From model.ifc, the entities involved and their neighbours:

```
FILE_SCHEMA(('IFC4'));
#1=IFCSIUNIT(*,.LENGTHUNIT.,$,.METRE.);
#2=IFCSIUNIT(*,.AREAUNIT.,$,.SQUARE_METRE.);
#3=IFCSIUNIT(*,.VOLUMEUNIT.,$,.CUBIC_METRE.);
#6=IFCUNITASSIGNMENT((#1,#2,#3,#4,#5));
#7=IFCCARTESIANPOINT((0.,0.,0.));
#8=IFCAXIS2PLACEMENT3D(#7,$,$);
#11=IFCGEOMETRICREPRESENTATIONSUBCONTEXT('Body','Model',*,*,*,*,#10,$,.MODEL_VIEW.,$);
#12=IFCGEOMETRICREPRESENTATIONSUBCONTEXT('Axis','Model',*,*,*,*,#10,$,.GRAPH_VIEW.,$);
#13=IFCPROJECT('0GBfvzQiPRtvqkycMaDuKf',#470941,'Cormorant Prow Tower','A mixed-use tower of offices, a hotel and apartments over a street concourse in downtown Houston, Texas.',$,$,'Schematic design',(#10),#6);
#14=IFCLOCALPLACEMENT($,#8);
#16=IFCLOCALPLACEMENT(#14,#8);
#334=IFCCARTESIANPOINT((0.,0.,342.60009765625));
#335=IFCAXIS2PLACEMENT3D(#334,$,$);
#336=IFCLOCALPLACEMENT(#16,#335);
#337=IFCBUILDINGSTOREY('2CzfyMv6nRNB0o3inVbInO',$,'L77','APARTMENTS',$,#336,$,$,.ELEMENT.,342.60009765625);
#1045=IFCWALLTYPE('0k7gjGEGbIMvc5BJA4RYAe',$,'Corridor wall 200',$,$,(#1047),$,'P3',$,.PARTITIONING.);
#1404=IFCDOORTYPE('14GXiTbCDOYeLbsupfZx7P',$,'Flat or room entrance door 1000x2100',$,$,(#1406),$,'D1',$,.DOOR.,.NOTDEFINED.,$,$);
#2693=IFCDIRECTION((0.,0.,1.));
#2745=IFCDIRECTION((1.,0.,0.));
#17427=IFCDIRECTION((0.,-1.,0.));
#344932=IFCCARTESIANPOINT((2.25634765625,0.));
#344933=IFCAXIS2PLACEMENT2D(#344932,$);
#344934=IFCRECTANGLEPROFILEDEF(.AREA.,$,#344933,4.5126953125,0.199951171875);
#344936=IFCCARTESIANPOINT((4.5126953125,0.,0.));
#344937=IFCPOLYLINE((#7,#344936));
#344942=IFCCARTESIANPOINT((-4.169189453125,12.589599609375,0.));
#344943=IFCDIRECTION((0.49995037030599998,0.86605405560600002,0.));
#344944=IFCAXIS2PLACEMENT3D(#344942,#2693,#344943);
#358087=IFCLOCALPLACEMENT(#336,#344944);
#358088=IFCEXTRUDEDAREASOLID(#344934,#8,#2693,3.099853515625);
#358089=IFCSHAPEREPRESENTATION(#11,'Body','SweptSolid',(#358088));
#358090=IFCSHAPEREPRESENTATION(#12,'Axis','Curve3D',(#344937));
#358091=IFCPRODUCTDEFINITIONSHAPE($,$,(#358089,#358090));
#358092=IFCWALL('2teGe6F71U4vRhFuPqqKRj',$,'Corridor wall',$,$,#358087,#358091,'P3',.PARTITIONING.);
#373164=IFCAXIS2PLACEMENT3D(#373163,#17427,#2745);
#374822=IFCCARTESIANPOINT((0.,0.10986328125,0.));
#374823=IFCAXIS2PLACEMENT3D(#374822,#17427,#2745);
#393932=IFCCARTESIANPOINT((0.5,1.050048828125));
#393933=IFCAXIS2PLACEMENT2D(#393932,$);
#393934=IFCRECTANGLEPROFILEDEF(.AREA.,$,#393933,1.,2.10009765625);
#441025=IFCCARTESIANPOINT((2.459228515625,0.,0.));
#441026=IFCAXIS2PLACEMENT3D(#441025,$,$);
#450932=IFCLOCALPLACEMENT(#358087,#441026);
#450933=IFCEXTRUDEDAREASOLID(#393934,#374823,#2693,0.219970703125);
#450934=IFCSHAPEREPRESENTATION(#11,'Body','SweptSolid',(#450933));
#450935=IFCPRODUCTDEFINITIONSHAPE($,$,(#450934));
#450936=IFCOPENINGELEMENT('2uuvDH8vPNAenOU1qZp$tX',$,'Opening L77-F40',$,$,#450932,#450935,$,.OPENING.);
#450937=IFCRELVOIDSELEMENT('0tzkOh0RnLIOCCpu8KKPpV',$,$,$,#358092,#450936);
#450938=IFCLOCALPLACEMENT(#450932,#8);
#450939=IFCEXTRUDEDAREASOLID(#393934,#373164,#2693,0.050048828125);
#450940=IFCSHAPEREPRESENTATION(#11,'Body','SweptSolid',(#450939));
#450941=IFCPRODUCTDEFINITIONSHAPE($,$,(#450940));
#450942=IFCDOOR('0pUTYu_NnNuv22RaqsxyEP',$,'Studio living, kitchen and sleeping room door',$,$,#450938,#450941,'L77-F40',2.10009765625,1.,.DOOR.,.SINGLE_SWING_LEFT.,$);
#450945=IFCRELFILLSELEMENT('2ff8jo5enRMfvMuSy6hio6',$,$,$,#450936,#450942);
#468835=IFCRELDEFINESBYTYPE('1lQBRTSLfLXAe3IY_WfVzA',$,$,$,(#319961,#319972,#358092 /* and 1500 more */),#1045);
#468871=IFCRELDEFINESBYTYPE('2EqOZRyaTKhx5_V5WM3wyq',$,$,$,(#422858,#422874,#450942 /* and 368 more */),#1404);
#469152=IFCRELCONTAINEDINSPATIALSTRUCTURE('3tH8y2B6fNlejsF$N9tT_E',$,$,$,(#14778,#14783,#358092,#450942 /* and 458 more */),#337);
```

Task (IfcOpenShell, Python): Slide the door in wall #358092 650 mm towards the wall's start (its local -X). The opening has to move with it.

```python
import ifcopenshell
import ifcopenshell.api.geometry
import ifcopenshell.util.placement

model = ifcopenshell.open("model.ifc")

door = model.by_id(450942)
opening = door.FillsVoids[0].RelatingOpeningElement
wall = opening.VoidsElements[0].RelatingBuildingElement

wall_matrix = ifcopenshell.util.placement.get_local_placement(wall.ObjectPlacement)
shift = wall_matrix[:3, 0] * -0.65
before = ifcopenshell.util.placement.get_local_placement(door.ObjectPlacement)[:3, 3].copy()

# The door is placed relative to its opening, so it follows when the opening moves.
matrix = ifcopenshell.util.placement.get_local_placement(opening.ObjectPlacement)
matrix[:3, 3] += shift
ifcopenshell.api.geometry.edit_object_placement(
    model, product=opening, matrix=matrix, is_si=False, should_transform_children=True
)

after = ifcopenshell.util.placement.get_local_placement(door.ObjectPlacement)[:3, 3]
print("door moved by", (after - before).round(3) + 0.0)

model.write("model-out.ifc")
```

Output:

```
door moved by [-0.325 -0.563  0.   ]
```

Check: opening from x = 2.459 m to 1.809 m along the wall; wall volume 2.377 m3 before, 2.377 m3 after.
